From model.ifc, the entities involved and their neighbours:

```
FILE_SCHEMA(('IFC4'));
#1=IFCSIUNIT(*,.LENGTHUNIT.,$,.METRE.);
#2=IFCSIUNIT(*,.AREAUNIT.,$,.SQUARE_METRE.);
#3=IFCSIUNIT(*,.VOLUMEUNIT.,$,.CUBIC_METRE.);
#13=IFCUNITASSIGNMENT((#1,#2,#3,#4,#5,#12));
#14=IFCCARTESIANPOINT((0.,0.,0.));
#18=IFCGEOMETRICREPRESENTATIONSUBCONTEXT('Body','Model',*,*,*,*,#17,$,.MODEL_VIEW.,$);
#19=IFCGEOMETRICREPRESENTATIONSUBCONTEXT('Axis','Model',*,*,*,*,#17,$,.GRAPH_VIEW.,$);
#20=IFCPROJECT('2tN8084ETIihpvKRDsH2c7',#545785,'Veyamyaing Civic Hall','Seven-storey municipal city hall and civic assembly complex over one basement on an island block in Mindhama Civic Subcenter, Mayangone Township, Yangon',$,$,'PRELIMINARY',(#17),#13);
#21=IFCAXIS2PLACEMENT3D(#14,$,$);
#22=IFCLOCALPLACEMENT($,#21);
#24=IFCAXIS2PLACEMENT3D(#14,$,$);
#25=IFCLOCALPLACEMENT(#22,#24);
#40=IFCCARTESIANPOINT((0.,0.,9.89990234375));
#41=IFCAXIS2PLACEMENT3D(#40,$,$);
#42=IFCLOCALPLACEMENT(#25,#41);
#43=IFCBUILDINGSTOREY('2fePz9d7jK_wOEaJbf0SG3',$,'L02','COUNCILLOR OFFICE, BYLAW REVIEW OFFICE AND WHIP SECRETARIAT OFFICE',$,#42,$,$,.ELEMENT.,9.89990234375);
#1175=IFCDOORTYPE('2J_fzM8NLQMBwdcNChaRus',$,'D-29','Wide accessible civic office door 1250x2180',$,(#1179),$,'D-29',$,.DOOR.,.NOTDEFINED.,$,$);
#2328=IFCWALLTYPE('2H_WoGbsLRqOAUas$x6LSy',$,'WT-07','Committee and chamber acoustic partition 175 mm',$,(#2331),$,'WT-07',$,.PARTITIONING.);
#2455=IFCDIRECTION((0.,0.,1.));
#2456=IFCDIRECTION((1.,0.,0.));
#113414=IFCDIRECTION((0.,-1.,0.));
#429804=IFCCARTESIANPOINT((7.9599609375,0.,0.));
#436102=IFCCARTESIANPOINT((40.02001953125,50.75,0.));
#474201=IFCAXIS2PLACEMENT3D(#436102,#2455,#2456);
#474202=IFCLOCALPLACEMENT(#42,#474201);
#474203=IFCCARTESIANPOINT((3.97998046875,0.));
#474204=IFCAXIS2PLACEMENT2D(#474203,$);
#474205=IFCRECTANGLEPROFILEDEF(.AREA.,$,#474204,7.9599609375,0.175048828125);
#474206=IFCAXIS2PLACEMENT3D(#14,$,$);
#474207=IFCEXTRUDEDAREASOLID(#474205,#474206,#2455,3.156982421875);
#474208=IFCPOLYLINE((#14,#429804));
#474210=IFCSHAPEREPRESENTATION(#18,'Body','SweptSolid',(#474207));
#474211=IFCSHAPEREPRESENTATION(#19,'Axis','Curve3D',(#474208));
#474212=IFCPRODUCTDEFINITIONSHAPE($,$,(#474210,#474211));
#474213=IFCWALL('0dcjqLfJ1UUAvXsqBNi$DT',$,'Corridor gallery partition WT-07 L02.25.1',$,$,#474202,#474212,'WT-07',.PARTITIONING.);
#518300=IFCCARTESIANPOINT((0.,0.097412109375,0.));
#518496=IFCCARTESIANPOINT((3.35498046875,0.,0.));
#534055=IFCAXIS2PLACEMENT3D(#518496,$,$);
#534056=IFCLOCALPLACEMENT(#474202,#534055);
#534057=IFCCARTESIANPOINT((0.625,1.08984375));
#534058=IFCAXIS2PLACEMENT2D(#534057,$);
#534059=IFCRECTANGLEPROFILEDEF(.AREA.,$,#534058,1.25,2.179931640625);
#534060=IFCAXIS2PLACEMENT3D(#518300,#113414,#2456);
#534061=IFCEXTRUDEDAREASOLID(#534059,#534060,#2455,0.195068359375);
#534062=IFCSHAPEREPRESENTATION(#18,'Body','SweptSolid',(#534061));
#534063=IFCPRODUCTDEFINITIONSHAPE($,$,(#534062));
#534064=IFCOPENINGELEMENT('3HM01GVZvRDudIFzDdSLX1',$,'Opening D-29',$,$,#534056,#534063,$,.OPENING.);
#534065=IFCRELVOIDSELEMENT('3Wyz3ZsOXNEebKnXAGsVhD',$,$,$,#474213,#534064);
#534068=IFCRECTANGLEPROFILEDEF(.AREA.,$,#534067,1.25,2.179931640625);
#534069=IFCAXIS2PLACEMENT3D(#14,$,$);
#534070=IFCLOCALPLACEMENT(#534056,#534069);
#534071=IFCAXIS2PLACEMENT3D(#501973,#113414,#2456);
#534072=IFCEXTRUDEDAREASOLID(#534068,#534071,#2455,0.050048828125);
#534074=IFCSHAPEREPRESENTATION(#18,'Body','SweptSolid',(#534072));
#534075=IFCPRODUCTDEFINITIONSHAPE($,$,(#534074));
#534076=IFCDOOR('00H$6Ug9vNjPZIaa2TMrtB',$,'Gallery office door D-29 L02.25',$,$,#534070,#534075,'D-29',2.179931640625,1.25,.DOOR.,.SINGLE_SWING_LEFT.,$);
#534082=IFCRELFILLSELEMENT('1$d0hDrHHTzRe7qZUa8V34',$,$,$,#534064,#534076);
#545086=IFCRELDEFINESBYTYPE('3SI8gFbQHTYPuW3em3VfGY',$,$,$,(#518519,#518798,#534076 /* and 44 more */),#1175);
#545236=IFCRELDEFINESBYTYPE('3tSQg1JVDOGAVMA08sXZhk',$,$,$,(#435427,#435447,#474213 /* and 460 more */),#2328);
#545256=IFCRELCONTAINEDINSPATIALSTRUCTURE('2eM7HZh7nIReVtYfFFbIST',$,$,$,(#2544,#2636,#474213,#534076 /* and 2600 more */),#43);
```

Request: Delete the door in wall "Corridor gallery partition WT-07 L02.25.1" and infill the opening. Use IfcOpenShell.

```python
import ifcopenshell
import ifcopenshell.api.feature
import ifcopenshell.api.root
import ifcopenshell.geom
import ifcopenshell.util.shape

model = ifcopenshell.open("model.ifc")
settings = ifcopenshell.geom.settings()


def volume(element):
    """Net volume in cubic metres, openings subtracted."""
    shape = ifcopenshell.geom.create_shape(settings, element)
    return ifcopenshell.util.shape.get_volume(shape.geometry)


door = model.by_guid("00H$6Ug9vNjPZIaa2TMrtB")
opening = door.FillsVoids[0].RelatingOpeningElement
wall = opening.VoidsElements[0].RelatingBuildingElement
before = volume(wall)

ifcopenshell.api.root.remove_product(model, product=door)
ifcopenshell.api.feature.remove_feature(model, feature=opening)

after = volume(wall)

print(f"wall volume {before:.3f} -> {after:.3f} m3")

model.write("model_rev.ifc")
```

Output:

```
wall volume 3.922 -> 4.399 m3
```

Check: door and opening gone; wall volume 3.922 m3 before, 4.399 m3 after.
